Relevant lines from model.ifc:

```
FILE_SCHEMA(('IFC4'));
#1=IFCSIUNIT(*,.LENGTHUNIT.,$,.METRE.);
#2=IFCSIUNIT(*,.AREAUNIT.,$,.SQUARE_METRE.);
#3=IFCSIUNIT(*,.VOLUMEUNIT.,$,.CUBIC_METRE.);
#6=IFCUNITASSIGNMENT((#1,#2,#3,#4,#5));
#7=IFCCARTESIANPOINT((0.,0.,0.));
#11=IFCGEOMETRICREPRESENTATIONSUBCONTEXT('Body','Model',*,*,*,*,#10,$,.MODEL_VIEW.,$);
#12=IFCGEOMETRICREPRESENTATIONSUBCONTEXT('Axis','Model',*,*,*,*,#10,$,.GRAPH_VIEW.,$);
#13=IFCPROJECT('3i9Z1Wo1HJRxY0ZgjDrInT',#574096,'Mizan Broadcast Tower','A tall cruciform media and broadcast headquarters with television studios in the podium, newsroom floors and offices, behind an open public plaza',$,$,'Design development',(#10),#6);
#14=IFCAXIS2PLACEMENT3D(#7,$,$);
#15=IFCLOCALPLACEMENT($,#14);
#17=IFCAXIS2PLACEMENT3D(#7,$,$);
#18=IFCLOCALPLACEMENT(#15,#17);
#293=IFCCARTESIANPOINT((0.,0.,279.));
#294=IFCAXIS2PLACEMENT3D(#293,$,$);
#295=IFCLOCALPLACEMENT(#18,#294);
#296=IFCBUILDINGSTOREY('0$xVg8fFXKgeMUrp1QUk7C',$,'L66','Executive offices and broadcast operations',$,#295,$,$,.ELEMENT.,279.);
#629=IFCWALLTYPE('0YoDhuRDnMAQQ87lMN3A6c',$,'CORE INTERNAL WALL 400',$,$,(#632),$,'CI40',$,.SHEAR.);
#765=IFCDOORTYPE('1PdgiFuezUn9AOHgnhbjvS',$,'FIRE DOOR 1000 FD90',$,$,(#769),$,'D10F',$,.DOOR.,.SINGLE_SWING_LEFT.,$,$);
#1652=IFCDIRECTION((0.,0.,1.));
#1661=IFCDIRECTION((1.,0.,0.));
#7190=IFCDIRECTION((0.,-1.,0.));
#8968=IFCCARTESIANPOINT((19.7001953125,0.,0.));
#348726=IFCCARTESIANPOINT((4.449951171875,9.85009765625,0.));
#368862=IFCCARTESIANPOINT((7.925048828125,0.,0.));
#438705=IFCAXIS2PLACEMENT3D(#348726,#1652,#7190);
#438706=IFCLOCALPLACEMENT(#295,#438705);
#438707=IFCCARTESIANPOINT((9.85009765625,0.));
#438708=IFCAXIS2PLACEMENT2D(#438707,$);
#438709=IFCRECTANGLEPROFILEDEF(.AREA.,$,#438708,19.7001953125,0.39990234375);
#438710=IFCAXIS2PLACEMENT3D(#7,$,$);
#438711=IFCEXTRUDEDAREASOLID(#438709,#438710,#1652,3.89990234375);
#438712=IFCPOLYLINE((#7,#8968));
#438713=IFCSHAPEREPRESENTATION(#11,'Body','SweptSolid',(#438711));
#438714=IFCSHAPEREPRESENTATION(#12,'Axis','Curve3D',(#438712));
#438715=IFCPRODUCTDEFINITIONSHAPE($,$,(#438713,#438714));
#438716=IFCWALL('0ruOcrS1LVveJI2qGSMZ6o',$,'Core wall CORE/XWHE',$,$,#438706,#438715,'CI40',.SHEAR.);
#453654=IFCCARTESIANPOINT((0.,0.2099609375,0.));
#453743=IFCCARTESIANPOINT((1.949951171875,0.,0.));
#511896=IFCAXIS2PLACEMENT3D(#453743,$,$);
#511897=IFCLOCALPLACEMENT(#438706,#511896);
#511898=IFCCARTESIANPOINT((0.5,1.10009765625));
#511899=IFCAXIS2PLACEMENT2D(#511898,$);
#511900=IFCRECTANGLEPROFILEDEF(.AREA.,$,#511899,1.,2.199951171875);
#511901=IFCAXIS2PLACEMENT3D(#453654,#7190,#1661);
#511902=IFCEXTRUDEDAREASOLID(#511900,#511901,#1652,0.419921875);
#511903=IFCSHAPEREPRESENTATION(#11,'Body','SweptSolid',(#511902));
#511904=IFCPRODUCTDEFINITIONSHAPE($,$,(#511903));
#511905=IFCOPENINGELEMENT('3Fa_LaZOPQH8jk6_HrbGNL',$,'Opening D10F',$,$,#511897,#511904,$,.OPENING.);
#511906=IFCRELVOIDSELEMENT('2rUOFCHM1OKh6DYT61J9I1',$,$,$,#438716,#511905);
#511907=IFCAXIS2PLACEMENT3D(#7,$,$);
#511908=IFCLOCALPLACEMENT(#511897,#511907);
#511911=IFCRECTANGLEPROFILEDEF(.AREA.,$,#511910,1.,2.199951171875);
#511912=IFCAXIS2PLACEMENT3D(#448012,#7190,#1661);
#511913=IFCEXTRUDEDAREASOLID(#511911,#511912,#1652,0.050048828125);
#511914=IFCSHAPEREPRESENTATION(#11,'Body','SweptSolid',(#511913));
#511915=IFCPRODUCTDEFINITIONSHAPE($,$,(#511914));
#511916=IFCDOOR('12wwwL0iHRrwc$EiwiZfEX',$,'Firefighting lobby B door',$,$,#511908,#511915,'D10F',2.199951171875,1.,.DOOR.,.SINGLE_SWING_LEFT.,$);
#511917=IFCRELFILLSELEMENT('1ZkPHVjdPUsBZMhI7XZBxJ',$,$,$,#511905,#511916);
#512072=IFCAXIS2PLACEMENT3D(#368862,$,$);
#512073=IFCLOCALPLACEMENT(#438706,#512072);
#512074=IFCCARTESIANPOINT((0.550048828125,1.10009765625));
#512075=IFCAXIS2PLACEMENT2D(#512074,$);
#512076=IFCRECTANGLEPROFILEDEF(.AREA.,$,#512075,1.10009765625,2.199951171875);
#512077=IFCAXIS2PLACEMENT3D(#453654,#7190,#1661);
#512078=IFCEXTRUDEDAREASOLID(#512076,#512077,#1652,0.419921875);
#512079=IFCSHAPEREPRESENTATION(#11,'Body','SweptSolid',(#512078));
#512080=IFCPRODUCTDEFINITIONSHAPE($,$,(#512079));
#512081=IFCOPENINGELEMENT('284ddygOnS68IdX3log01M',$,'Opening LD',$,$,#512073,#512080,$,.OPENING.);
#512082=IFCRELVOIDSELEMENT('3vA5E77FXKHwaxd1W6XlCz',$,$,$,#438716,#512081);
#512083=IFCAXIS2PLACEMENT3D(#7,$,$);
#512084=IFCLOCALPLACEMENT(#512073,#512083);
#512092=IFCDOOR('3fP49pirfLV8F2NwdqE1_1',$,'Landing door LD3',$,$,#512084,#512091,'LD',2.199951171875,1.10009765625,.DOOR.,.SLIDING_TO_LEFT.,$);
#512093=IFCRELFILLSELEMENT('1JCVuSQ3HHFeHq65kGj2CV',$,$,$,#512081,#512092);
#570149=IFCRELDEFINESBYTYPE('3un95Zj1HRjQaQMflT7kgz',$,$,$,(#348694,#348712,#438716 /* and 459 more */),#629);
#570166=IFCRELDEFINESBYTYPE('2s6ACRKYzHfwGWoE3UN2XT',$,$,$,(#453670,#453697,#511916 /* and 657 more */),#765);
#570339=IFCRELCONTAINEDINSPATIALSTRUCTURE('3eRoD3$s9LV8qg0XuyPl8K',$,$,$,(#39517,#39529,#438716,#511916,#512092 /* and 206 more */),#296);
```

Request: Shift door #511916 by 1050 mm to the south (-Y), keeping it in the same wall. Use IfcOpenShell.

```python
import ifcopenshell
import ifcopenshell.api.geometry
import ifcopenshell.util.placement

model = ifcopenshell.open("model.ifc")

door = model.by_guid("12wwwL0iHRrwc$EiwiZfEX")
opening = door.FillsVoids[0].RelatingOpeningElement
wall = opening.VoidsElements[0].RelatingBuildingElement

wall_matrix = ifcopenshell.util.placement.get_local_placement(wall.ObjectPlacement)
shift = wall_matrix[:3, 0] * 1.05
before = ifcopenshell.util.placement.get_local_placement(door.ObjectPlacement)[:3, 3].copy()

# The door is placed relative to its opening, so it follows when the opening moves.
matrix = ifcopenshell.util.placement.get_local_placement(opening.ObjectPlacement)
matrix[:3, 3] += shift
ifcopenshell.api.geometry.edit_object_placement(
    model, product=opening, matrix=matrix, is_si=False, should_transform_children=True
)

after = ifcopenshell.util.placement.get_local_placement(door.ObjectPlacement)[:3, 3]
print("door moved by", (after - before).round(3) + 0.0)

model.write("model-out.ifc")
```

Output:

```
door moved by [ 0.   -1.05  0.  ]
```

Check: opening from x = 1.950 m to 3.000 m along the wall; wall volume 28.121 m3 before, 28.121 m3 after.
